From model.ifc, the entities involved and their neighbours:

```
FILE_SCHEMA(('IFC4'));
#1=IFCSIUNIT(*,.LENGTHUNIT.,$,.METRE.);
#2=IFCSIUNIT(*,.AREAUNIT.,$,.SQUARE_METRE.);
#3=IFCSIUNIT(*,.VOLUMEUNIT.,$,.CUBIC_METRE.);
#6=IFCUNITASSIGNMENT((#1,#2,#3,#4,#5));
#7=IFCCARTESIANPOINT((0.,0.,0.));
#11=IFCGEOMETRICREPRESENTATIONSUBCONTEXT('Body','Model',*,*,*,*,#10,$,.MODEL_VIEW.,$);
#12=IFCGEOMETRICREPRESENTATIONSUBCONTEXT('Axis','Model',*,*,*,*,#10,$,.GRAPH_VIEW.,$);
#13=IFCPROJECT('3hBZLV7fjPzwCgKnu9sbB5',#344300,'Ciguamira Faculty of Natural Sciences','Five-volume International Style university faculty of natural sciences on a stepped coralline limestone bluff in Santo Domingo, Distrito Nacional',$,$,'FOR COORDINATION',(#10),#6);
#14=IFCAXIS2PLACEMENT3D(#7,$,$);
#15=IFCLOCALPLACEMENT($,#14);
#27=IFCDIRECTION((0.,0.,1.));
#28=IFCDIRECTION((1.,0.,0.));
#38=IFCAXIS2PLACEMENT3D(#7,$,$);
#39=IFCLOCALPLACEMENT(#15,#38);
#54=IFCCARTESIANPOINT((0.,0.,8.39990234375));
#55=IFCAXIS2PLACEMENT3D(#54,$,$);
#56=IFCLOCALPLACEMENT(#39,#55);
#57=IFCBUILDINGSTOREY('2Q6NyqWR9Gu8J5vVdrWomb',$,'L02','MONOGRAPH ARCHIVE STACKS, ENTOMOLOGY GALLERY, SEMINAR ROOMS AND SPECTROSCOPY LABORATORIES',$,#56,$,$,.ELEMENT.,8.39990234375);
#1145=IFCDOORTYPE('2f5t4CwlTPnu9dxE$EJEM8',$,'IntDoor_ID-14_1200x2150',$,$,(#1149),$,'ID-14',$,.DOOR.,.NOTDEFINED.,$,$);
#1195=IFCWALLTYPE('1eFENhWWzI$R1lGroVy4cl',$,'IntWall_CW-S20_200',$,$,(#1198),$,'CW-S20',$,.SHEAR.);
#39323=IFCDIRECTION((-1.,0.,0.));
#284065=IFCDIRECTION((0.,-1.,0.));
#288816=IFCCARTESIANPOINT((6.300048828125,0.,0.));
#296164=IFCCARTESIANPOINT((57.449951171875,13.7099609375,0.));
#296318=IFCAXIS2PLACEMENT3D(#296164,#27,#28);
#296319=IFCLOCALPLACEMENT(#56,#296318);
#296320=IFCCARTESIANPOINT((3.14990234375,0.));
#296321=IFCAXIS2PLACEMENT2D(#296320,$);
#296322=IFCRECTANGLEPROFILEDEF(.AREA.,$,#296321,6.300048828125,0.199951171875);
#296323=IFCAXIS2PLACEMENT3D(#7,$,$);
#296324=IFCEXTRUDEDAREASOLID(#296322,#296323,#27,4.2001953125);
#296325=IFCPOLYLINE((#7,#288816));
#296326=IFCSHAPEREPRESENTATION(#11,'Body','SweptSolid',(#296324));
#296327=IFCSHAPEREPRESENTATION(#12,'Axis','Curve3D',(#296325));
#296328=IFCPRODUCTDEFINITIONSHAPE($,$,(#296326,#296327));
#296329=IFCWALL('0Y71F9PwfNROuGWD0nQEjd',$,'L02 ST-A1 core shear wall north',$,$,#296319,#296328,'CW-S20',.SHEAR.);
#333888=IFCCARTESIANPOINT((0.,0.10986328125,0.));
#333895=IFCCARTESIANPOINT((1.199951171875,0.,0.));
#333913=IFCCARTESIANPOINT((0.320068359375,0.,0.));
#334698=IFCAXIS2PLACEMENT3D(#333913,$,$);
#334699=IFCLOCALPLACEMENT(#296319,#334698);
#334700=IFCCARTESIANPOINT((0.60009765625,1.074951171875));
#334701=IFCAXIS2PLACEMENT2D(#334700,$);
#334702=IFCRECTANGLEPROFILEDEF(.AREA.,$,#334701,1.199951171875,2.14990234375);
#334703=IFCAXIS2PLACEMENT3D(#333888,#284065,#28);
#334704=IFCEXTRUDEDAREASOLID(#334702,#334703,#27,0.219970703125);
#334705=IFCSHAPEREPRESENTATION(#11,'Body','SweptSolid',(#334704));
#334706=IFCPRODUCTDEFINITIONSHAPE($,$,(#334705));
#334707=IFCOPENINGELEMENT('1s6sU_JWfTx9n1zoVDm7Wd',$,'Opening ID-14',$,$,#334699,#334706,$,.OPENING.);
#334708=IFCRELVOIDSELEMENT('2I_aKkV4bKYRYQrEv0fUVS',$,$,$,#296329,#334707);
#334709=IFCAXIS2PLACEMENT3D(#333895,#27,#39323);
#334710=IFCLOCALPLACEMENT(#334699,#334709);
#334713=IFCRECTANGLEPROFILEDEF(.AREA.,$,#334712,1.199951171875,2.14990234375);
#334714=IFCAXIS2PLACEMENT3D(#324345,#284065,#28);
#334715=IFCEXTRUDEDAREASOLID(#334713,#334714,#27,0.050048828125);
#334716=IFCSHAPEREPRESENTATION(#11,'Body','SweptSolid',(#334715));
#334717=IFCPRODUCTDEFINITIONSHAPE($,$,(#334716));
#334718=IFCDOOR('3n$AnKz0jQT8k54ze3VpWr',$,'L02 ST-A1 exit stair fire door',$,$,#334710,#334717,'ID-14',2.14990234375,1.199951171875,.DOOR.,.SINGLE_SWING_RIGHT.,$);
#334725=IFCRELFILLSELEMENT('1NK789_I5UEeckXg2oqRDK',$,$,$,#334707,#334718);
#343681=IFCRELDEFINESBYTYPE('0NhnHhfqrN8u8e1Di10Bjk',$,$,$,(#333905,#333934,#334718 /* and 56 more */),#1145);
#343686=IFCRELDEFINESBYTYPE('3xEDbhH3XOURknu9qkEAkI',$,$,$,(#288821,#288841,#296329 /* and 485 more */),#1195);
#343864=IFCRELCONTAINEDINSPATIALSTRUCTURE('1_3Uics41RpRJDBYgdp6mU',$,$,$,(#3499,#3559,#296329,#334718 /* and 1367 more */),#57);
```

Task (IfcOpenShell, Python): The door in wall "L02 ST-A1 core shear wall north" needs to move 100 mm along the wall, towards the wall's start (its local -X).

```python
import ifcopenshell
import ifcopenshell.api.geometry
import ifcopenshell.util.placement
import ifcopenshell.util.unit

model = ifcopenshell.open("model.ifc")
unit_scale = ifcopenshell.util.unit.calculate_unit_scale(model)

door = model.by_guid("3n$AnKz0jQT8k54ze3VpWr")
opening = door.FillsVoids[0].RelatingOpeningElement
wall = opening.VoidsElements[0].RelatingBuildingElement

wall_matrix = ifcopenshell.util.placement.get_local_placement(wall.ObjectPlacement)
shift = wall_matrix[:3, 0] * -0.1 / unit_scale
before = ifcopenshell.util.placement.get_local_placement(door.ObjectPlacement)[:3, 3].copy()

# The door is placed relative to its opening, so it follows when the opening moves.
matrix = ifcopenshell.util.placement.get_local_placement(opening.ObjectPlacement)
matrix[:3, 3] += shift
ifcopenshell.api.geometry.edit_object_placement(
    model, product=opening, matrix=matrix, is_si=False, should_transform_children=True
)

after = ifcopenshell.util.placement.get_local_placement(door.ObjectPlacement)[:3, 3]
print("door moved by", (after - before).round(3) + 0.0)

model.write("model_updated.ifc")
```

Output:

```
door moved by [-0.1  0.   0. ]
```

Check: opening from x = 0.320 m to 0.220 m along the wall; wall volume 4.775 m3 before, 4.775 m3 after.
